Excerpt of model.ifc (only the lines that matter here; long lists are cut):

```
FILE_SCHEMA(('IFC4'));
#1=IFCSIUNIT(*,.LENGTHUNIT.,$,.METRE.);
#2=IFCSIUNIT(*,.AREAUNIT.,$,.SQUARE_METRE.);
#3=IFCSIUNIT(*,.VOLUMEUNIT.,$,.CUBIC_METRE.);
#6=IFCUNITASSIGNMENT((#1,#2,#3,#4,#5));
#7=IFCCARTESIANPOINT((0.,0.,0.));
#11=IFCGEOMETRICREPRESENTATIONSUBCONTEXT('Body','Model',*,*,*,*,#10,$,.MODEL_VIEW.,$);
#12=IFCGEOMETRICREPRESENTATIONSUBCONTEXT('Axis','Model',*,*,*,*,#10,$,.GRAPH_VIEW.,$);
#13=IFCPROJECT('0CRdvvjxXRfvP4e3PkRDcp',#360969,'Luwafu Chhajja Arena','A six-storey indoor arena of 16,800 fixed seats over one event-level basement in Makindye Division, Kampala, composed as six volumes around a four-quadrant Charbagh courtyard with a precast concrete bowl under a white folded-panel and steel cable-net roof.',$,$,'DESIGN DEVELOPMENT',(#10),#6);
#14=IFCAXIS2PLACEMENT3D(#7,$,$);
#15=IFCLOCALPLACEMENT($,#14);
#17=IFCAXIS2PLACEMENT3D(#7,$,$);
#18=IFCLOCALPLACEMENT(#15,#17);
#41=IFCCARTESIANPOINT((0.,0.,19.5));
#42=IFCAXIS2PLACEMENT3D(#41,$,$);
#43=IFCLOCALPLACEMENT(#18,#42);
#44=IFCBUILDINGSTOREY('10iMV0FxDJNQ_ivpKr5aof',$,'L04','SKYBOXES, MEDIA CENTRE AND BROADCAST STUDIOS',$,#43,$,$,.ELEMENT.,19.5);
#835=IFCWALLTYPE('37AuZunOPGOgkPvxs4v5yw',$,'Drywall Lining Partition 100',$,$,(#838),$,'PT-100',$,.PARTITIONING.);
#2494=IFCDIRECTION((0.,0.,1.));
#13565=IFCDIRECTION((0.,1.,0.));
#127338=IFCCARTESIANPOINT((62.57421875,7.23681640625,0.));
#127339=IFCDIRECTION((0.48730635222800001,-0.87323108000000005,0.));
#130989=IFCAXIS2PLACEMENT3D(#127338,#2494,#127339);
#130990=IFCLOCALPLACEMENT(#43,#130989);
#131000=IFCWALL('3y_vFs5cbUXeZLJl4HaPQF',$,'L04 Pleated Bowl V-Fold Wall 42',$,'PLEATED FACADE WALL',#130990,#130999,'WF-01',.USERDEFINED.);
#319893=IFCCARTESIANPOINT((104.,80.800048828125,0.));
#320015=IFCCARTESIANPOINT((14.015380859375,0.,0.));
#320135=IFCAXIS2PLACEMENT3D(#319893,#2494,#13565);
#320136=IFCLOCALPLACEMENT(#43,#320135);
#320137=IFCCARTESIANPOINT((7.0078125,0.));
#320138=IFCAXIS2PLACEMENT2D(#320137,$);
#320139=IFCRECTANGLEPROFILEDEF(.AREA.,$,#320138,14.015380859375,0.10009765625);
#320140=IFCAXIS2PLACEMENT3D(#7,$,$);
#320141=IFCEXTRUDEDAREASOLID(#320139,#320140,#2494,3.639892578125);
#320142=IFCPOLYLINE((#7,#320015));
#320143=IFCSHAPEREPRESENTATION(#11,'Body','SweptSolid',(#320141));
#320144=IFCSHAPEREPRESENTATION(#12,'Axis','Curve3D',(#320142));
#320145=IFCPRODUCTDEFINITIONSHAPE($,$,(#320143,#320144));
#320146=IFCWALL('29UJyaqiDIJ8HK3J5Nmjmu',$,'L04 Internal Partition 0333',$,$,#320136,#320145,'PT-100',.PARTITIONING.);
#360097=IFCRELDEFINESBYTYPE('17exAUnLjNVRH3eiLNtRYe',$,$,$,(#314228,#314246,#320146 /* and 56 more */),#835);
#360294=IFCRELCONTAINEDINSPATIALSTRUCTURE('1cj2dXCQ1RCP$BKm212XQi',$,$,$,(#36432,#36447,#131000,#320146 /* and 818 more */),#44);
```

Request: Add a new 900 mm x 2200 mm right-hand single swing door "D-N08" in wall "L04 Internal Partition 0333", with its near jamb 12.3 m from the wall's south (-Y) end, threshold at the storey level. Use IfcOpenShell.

```python
import numpy as np
import ifcopenshell
import ifcopenshell.api.feature
import ifcopenshell.api.geometry
import ifcopenshell.api.root
import ifcopenshell.api.spatial
import ifcopenshell.geom
import ifcopenshell.util.element
import ifcopenshell.util.placement
import ifcopenshell.util.representation
import ifcopenshell.util.shape
import ifcopenshell.util.unit

model = ifcopenshell.open("model.ifc")
unit_scale = ifcopenshell.util.unit.calculate_unit_scale(model)
settings = ifcopenshell.geom.settings()


def volume(element):
    """Net volume in cubic metres, openings subtracted."""
    shape = ifcopenshell.geom.create_shape(settings, element)
    return ifcopenshell.util.shape.get_volume(shape.geometry)


wall = model.by_guid("29UJyaqiDIJ8HK3J5Nmjmu")
storey = ifcopenshell.util.element.get_container(wall, ifc_class="IfcBuildingStorey")
context = ifcopenshell.util.representation.get_context(model, "Model", "Body", "MODEL_VIEW")
before = volume(wall)

width, height, from_end, sill = 0.9, 2.2, 12.3, 0.0  # metres

# The wall runs along its own X axis, and the end named is its -X end.
wall_shape = ifcopenshell.geom.create_shape(settings, wall)
x, y, z = ifcopenshell.util.shape.get_vertices(wall_shape.geometry).T
start = x.min() + from_end
face, thickness = float(y.min()), float(y.max() - y.min())
wall_matrix = ifcopenshell.util.placement.get_local_placement(wall.ObjectPlacement)
level = ifcopenshell.util.placement.get_local_placement(storey.ObjectPlacement)[2, 3]


def in_wall(x, y):
    """Placement at x, y metres in the wall's axes, at sill height."""
    matrix = wall_matrix.copy()
    matrix[:, 3] = wall_matrix @ np.array([x / unit_scale, y / unit_scale, 0.0, 1.0])
    matrix[2, 3] = level + sill / unit_scale
    return matrix


# Opening: a box that overshoots both wall faces by 50 mm.
opening = ifcopenshell.api.root.create_entity(model, ifc_class="IfcOpeningElement", predefined_type="OPENING")
box = ifcopenshell.api.geometry.add_wall_representation(
    model, context=context, length=width, height=height, thickness=thickness + 0.1
)
ifcopenshell.api.geometry.assign_representation(model, product=opening, representation=box)
ifcopenshell.api.geometry.edit_object_placement(model, product=opening, matrix=in_wall(start, face - 0.05), is_si=False)
ifcopenshell.api.feature.add_feature(model, feature=opening, element=wall)

door = ifcopenshell.api.root.create_entity(model, ifc_class="IfcDoor", name="D-N08", predefined_type="DOOR")
door.OverallWidth, door.OverallHeight = width / unit_scale, height / unit_scale
door.OperationType = "SINGLE_SWING_RIGHT"
body = ifcopenshell.api.geometry.add_door_representation(
    model,
    context=context,
    overall_width=door.OverallWidth,
    overall_height=door.OverallHeight,
    operation_type="SINGLE_SWING_RIGHT",
    lining_properties={"LiningDepth": thickness / unit_scale, "ThresholdDepth": thickness / unit_scale},
)
ifcopenshell.api.geometry.assign_representation(model, product=door, representation=body)
ifcopenshell.api.spatial.assign_container(model, products=[door], relating_structure=storey)
ifcopenshell.api.feature.add_filling(model, opening=opening, element=door)

# The lining spans the wall, so the door starts at the wall face.
ifcopenshell.api.geometry.edit_object_placement(model, product=door, matrix=in_wall(start, face), is_si=False)

after = volume(wall)

print(f"wall volume {before:.3f} -> {after:.3f} m3")

model.write("model_updated.ifc")
```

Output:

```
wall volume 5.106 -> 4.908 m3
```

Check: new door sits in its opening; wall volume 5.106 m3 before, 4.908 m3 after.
